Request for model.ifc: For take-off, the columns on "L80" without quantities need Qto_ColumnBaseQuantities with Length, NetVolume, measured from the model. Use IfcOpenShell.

First a look at what the model holds.

```python
import ifcopenshell
import ifcopenshell.util.element
import ifcopenshell.util.unit

model = ifcopenshell.open("model.ifc")
print(model.schema)
for unit_type in ("LENGTHUNIT", "AREAUNIT", "VOLUMEUNIT"):
    print(unit_type, ifcopenshell.util.unit.calculate_unit_scale(model, unit_type))
storey = next(s for s in model.by_type("IfcBuildingStorey") if s.Name == "L80")
columns = [e for e in ifcopenshell.util.element.get_decomposition(storey) if e.is_a("IfcColumn")]
for e in sorted(columns, key=lambda e: e.id()):
    print(e.id(), e.is_a(), e.Name, list(ifcopenshell.util.element.get_psets(e, qtos_only=True)), sep=" | ")
```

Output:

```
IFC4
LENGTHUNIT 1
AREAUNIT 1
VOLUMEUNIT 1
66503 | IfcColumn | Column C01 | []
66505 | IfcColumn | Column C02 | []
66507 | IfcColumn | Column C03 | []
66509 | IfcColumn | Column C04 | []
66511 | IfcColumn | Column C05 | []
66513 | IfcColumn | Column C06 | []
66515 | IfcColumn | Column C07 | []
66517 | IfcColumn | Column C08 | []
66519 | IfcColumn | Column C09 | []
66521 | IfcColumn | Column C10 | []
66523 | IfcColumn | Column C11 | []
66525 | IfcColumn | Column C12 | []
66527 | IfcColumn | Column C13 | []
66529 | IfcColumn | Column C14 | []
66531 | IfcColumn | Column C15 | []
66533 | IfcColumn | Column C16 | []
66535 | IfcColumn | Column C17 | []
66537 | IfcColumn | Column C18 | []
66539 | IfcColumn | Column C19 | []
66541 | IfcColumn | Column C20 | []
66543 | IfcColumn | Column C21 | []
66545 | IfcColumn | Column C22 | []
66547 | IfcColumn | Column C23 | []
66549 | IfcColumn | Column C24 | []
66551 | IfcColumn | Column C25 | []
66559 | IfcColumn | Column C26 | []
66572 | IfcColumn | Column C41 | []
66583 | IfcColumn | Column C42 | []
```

```python
import ifcopenshell
import ifcopenshell.api.pset
import ifcopenshell.geom
import ifcopenshell.util.element
import ifcopenshell.util.shape
import ifcopenshell.util.unit

model = ifcopenshell.open("model.ifc")
unit_scale = ifcopenshell.util.unit.calculate_unit_scale(model)
volume_scale = ifcopenshell.util.unit.calculate_unit_scale(model, "VOLUMEUNIT")
settings = ifcopenshell.geom.settings()

storey = next(s for s in model.by_type("IfcBuildingStorey") if s.Name == "L80")
columns = [e for e in ifcopenshell.util.element.get_decomposition(storey) if e.is_a("IfcColumn")]

for e in sorted(columns, key=lambda e: e.id()):
    if ifcopenshell.util.element.get_psets(e, qtos_only=True, should_inherit=False):
        continue
    # Geometry comes back in metres, in the element's own axes.
    shape = ifcopenshell.geom.create_shape(settings, e)
    values = {
        "Length": ifcopenshell.util.shape.get_z(shape.geometry) / unit_scale,
        "NetVolume": ifcopenshell.util.shape.get_volume(shape.geometry) / volume_scale,
    }
    qto = ifcopenshell.api.pset.add_qto(model, product=e, name="Qto_ColumnBaseQuantities")
    ifcopenshell.api.pset.edit_qto(model, qto=qto, properties=values)
    print(e.id(), {k: round(v, 3) for k, v in values.items()})

model.write("model-out.ifc")
```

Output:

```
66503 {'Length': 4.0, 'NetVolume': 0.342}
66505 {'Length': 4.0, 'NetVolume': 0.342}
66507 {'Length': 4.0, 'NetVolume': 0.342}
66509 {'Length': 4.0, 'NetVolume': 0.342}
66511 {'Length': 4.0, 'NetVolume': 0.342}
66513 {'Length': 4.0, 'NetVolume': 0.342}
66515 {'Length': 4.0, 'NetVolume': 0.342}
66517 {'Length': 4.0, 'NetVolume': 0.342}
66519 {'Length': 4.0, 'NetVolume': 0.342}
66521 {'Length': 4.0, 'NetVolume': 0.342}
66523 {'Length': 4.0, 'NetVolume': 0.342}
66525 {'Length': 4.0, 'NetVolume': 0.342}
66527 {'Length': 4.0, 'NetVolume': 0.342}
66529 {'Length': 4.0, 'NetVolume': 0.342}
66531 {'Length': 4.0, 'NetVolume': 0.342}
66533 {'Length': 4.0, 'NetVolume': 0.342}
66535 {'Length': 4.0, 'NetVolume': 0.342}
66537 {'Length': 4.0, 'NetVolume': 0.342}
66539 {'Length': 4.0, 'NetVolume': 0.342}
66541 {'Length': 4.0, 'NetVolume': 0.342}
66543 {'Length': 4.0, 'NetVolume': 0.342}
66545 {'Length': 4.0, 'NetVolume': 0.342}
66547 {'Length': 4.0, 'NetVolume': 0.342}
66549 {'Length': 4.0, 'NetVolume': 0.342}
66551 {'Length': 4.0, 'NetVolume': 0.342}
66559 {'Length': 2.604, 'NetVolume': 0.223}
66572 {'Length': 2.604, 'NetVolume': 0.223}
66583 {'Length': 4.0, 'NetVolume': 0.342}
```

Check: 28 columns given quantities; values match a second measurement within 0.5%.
